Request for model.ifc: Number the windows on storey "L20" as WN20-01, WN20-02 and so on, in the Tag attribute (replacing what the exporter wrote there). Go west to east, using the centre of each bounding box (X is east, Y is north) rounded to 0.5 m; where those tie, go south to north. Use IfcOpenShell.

First a look at what the model holds.

```python
import ifcopenshell
import ifcopenshell.util.element
import ifcopenshell.util.placement

model = ifcopenshell.open("model.ifc")
print(model.schema)
storey = next(s for s in model.by_type("IfcBuildingStorey") if s.Name == "L20")
windows = [e for e in ifcopenshell.util.element.get_decomposition(storey) if e.is_a("IfcWindow")]
for e in sorted(windows, key=lambda e: e.id()):
    origin = ifcopenshell.util.placement.get_local_placement(e.ObjectPlacement)[:3, 3]
    print(e.id(), e.Tag, e.Name, origin.round(2) + 0.0, sep=" | ")
```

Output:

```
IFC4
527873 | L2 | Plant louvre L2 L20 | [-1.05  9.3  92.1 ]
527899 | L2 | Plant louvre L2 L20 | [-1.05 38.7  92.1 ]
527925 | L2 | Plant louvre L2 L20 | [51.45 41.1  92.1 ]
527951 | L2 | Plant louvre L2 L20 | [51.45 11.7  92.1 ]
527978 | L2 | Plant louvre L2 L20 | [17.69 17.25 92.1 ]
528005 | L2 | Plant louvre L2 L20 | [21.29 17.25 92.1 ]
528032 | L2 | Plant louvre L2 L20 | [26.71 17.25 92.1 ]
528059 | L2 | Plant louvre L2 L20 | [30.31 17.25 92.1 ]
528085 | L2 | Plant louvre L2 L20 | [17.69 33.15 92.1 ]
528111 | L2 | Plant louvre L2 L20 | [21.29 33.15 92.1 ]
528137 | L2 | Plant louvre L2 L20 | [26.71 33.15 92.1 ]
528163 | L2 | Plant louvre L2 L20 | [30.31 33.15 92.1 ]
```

```python
import ifcopenshell
import ifcopenshell.geom
import ifcopenshell.util.element
import ifcopenshell.util.shape

model = ifcopenshell.open("model.ifc")
settings = ifcopenshell.geom.settings()
settings.set("use-world-coords", True)


def centre(element):
    shape = ifcopenshell.geom.create_shape(settings, element)
    return ifcopenshell.util.shape.get_bbox_centroid(shape.geometry)


storey = next(s for s in model.by_type("IfcBuildingStorey") if s.Name == "L20")
windows = [e for e in ifcopenshell.util.element.get_decomposition(storey) if e.is_a("IfcWindow")]

# Insertion points can sit at a corner or the storey origin, so sort by the geometry (in metres).
centres = {e: centre(e) for e in windows}
windows.sort(key=lambda e: (round(centres[e][0] / 0.5), centres[e][1]))

for i, e in enumerate(windows, start=1):
    number = f"WN20-{i:02d}"
    e.Tag = number
    print(e.id(), number)

model.write("model_v2.ifc")
```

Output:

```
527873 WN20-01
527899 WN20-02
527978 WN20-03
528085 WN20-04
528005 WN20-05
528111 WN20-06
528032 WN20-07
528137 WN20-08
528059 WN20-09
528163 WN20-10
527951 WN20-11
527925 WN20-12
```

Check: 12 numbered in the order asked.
